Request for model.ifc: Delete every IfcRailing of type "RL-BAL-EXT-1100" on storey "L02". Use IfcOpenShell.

First a look at what the model holds.

```python
import ifcopenshell
import ifcopenshell.util.element

model = ifcopenshell.open("model.ifc")
print(model.schema)
storey = next(s for s in model.by_type("IfcBuildingStorey") if s.Name == "L02")
railings = [e for e in ifcopenshell.util.element.get_decomposition(storey) if e.is_a("IfcRailing")]
seen = {}
for e in railings:
    element_type = ifcopenshell.util.element.get_type(e)
    name = element_type.Name if element_type not in (None, e) else None
    seen[name] = seen.get(name, 0) + 1
for name, count in sorted(seen.items(), key=str):
    print(count, "x", name)
```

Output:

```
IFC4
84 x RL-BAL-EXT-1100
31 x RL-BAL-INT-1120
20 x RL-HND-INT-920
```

```python
import ifcopenshell
import ifcopenshell.api.root
import ifcopenshell.util.element

model = ifcopenshell.open("model.ifc")

storey = next(s for s in model.by_type("IfcBuildingStorey") if s.Name == "L02")
railings = [e for e in ifcopenshell.util.element.get_decomposition(storey) if e.is_a("IfcRailing")]
targets = [e for e in railings if (t := ifcopenshell.util.element.get_type(e)) not in (None, e) and t.Name == "RL-BAL-EXT-1100"]

for e in targets:
    ifcopenshell.api.root.remove_product(model, product=e)
print(len(targets), "removed")

model.write("model_updated.ifc")
```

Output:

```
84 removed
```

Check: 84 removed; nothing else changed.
